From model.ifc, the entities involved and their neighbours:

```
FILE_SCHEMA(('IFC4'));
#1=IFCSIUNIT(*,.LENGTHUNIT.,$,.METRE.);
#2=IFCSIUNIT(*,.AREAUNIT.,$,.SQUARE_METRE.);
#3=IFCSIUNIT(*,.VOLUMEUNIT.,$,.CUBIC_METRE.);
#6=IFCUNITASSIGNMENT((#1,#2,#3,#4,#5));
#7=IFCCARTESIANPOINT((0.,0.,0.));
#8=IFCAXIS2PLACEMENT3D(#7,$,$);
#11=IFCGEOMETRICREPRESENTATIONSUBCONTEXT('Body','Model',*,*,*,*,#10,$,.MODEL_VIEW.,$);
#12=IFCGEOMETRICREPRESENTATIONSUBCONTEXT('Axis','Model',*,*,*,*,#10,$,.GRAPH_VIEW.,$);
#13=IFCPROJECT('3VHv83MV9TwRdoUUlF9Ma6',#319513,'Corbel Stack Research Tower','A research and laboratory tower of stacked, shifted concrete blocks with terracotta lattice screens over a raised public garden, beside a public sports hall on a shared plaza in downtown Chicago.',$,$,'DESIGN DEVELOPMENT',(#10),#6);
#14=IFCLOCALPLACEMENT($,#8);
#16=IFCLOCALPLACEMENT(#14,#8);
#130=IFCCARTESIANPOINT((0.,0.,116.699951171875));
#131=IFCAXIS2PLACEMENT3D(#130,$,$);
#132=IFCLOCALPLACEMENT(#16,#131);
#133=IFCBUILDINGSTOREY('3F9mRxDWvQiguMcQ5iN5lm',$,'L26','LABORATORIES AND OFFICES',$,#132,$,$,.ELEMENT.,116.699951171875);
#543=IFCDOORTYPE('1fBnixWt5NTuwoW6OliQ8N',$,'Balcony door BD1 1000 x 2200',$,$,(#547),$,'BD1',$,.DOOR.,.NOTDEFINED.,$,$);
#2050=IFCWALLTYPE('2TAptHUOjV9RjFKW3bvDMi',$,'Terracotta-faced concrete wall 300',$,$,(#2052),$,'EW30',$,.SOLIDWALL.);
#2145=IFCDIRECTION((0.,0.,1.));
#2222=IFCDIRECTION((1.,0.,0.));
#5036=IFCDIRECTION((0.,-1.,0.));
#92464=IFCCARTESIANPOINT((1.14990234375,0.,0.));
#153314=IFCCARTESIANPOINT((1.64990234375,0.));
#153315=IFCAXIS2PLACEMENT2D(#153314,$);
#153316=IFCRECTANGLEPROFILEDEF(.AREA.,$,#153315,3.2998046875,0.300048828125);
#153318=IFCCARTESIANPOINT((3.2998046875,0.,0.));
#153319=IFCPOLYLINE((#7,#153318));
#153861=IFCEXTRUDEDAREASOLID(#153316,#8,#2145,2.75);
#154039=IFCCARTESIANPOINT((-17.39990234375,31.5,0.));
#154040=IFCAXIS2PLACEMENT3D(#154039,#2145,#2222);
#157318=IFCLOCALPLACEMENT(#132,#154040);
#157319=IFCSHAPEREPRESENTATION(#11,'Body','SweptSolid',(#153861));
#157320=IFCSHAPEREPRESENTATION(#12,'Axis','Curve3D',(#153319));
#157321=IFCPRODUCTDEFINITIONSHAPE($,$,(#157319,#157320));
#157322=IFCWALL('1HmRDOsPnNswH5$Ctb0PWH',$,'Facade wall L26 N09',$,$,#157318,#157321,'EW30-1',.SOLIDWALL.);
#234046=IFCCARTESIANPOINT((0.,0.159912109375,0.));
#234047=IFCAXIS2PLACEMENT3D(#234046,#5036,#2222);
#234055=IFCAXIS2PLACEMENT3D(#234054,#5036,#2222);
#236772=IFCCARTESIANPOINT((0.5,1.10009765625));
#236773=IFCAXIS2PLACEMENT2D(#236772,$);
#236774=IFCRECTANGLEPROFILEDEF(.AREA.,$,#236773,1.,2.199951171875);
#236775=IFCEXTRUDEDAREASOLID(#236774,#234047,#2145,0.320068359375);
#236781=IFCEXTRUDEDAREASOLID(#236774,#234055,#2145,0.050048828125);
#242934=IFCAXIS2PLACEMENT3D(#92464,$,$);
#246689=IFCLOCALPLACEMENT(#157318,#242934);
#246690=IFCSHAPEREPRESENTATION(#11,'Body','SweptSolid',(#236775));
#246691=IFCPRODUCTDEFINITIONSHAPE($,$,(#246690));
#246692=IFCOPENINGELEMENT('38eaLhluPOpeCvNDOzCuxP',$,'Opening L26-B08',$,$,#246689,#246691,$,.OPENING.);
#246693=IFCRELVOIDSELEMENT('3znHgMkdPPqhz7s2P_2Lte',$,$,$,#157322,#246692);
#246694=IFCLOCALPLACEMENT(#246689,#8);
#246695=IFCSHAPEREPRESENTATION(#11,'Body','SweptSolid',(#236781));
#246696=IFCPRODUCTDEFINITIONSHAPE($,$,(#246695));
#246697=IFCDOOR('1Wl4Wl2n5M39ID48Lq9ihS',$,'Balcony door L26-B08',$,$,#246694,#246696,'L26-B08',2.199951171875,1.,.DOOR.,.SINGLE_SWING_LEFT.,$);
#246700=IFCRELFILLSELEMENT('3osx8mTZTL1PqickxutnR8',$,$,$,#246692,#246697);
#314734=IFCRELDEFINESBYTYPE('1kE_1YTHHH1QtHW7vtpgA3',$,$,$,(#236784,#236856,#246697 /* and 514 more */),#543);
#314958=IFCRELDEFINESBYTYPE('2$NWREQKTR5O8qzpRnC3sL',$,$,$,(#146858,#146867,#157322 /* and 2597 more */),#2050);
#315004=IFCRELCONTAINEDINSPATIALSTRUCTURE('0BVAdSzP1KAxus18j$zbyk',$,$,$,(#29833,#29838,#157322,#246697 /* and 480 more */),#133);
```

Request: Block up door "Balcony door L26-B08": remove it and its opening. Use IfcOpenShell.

```python
import ifcopenshell
import ifcopenshell.api.feature
import ifcopenshell.api.root
import ifcopenshell.geom
import ifcopenshell.util.shape

model = ifcopenshell.open("model.ifc")
settings = ifcopenshell.geom.settings()


def volume(element):
    """Net volume in cubic metres, openings subtracted."""
    shape = ifcopenshell.geom.create_shape(settings, element)
    return ifcopenshell.util.shape.get_volume(shape.geometry)


door = model.by_guid("1Wl4Wl2n5M39ID48Lq9ihS")
opening = door.FillsVoids[0].RelatingOpeningElement
wall = opening.VoidsElements[0].RelatingBuildingElement
before = volume(wall)

ifcopenshell.api.root.remove_product(model, product=door)
ifcopenshell.api.feature.remove_feature(model, feature=opening)

after = volume(wall)

print(f"wall volume {before:.3f} -> {after:.3f} m3")

model.write("model-out.ifc")
```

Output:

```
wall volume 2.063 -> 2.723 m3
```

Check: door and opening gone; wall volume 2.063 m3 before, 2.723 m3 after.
